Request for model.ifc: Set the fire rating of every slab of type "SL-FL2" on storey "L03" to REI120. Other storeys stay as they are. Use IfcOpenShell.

First a look at what the model holds.

```python
import ifcopenshell
import ifcopenshell.util.element

model = ifcopenshell.open("model.ifc")
print(model.schema)
storey = next(s for s in model.by_type("IfcBuildingStorey") if s.Name == "L03")
slabs = [e for e in ifcopenshell.util.element.get_decomposition(storey) if e.is_a("IfcSlab")]
seen = {}
for e in slabs:
    element_type = ifcopenshell.util.element.get_type(e)
    key = (element_type.Name if element_type != e and element_type else None, ifcopenshell.util.element.get_pset(e, "Pset_SlabCommon", "FireRating"))
    seen[key] = seen.get(key, 0) + 1
for (name, value), count in sorted(seen.items(), key=str):
    print(count, "x", name, "|", value)
```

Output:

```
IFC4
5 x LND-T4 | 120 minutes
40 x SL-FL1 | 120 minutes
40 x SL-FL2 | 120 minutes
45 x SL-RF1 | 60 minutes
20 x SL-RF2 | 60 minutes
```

```python
import ifcopenshell
import ifcopenshell.api.pset
import ifcopenshell.util.element

model = ifcopenshell.open("model.ifc")

storey = next(s for s in model.by_type("IfcBuildingStorey") if s.Name == "L03")
slabs = [e for e in ifcopenshell.util.element.get_decomposition(storey) if e.is_a("IfcSlab")]

count = 0
for e in slabs:
    element_type = ifcopenshell.util.element.get_type(e)
    if element_type in (None, e) or element_type.Name != "SL-FL2":
        continue
    # add_pset returns the element's existing set when there is one.
    pset = ifcopenshell.api.pset.add_pset(model, product=e, name="Pset_SlabCommon")
    ifcopenshell.api.pset.edit_pset(model, pset=pset, properties={"FireRating": "REI120"})
    count += 1

print(count, "slabs updated")

model.write("model_edited.ifc")
```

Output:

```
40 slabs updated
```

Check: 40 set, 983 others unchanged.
